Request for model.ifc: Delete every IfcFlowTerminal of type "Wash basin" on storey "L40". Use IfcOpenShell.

First a look at what the model holds.

```python
import ifcopenshell
import ifcopenshell.util.element

model = ifcopenshell.open("model.ifc")
print(model.schema)
storey = next(s for s in model.by_type("IfcBuildingStorey") if s.Name == "L40")
terminals = [e for e in ifcopenshell.util.element.get_decomposition(storey) if e.is_a("IfcFlowTerminal")]
seen = {}
for e in terminals:
    element_type = ifcopenshell.util.element.get_type(e)
    name = element_type.Name if element_type not in (None, e) else None
    seen[name] = seen.get(name, 0) + 1
for name, count in sorted(seen.items(), key=str):
    print(count, "x", name)
```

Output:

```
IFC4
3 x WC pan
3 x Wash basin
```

```python
import ifcopenshell
import ifcopenshell.api.root
import ifcopenshell.util.element

model = ifcopenshell.open("model.ifc")

storey = next(s for s in model.by_type("IfcBuildingStorey") if s.Name == "L40")
terminals = [e for e in ifcopenshell.util.element.get_decomposition(storey) if e.is_a("IfcFlowTerminal")]
targets = [e for e in terminals if (t := ifcopenshell.util.element.get_type(e)) not in (None, e) and t.Name == "Wash basin"]

for e in targets:
    ifcopenshell.api.root.remove_product(model, product=e)
print(len(targets), "removed")

model.write("model_updated.ifc")
```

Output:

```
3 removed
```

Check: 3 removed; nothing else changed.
